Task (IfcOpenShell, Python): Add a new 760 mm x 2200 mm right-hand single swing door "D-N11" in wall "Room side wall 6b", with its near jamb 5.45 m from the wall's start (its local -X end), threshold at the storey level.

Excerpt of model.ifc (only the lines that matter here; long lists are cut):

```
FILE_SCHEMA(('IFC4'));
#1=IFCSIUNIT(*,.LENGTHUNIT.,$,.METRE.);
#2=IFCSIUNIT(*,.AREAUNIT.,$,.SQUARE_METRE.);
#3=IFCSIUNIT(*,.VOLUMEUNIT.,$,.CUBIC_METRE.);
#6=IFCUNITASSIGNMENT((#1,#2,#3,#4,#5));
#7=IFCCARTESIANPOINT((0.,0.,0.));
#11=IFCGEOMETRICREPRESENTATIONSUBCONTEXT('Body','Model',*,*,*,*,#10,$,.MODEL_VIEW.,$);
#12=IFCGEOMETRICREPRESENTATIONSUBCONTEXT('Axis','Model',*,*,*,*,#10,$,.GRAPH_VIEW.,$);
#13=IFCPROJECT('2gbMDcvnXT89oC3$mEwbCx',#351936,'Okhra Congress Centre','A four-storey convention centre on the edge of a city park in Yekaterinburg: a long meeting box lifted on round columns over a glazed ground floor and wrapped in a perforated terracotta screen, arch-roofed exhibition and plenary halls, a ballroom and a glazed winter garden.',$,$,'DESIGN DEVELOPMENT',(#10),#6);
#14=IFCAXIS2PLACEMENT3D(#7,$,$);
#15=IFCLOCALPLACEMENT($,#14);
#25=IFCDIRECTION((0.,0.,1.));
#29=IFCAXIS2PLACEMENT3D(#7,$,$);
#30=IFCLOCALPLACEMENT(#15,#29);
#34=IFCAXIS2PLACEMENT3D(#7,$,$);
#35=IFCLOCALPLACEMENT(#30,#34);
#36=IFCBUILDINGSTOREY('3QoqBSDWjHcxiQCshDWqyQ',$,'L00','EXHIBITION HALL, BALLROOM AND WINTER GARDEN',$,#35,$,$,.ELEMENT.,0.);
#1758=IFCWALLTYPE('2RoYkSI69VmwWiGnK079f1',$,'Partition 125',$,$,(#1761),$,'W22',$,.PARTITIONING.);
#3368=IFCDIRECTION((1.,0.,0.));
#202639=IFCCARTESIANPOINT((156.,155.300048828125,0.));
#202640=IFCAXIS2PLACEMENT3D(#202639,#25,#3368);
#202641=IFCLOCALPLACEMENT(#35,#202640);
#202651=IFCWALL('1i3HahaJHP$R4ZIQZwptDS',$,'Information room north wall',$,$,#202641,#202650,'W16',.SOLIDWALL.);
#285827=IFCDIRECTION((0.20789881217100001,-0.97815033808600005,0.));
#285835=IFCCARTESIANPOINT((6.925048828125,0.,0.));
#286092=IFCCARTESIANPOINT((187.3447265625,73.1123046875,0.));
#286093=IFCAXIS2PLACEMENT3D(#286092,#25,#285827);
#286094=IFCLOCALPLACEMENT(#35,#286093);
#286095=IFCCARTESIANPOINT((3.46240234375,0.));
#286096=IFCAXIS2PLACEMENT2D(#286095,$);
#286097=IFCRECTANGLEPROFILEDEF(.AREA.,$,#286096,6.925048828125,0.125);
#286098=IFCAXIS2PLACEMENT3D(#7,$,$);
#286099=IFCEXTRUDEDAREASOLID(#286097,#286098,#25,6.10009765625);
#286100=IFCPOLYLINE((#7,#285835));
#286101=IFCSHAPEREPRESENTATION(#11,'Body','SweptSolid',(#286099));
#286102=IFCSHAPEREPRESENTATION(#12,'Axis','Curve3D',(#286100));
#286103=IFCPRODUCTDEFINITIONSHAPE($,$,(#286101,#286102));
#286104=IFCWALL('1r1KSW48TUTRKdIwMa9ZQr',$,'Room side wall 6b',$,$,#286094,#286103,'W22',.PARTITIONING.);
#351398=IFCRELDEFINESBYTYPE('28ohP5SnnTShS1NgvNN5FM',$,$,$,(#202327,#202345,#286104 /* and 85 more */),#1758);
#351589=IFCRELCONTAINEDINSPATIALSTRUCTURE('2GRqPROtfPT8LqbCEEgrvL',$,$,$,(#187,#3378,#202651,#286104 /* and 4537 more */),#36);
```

```python
import numpy as np
import ifcopenshell
import ifcopenshell.api.feature
import ifcopenshell.api.geometry
import ifcopenshell.api.root
import ifcopenshell.api.spatial
import ifcopenshell.geom
import ifcopenshell.util.element
import ifcopenshell.util.placement
import ifcopenshell.util.representation
import ifcopenshell.util.shape
import ifcopenshell.util.unit

model = ifcopenshell.open("model.ifc")
unit_scale = ifcopenshell.util.unit.calculate_unit_scale(model)
settings = ifcopenshell.geom.settings()


def volume(element):
    """Net volume in cubic metres, openings subtracted."""
    shape = ifcopenshell.geom.create_shape(settings, element)
    return ifcopenshell.util.shape.get_volume(shape.geometry)


wall = model.by_guid("1r1KSW48TUTRKdIwMa9ZQr")
storey = ifcopenshell.util.element.get_container(wall, ifc_class="IfcBuildingStorey")
context = ifcopenshell.util.representation.get_context(model, "Model", "Body", "MODEL_VIEW")
before = volume(wall)

width, height, from_end, sill = 0.76, 2.2, 5.45, 0.0  # metres

# The wall runs along its own X axis, and the end named is its -X end.
wall_shape = ifcopenshell.geom.create_shape(settings, wall)
x, y, z = ifcopenshell.util.shape.get_vertices(wall_shape.geometry).T
start = x.min() + from_end
face, thickness = float(y.min()), float(y.max() - y.min())
wall_matrix = ifcopenshell.util.placement.get_local_placement(wall.ObjectPlacement)
level = ifcopenshell.util.placement.get_local_placement(storey.ObjectPlacement)[2, 3]


def in_wall(x, y):
    """Placement at x, y metres in the wall's axes, at sill height."""
    matrix = wall_matrix.copy()
    matrix[:, 3] = wall_matrix @ np.array([x / unit_scale, y / unit_scale, 0.0, 1.0])
    matrix[2, 3] = level + sill / unit_scale
    return matrix


# Opening: a box that overshoots both wall faces by 50 mm.
opening = ifcopenshell.api.root.create_entity(model, ifc_class="IfcOpeningElement", predefined_type="OPENING")
box = ifcopenshell.api.geometry.add_wall_representation(
    model, context=context, length=width, height=height, thickness=thickness + 0.1
)
ifcopenshell.api.geometry.assign_representation(model, product=opening, representation=box)
ifcopenshell.api.geometry.edit_object_placement(model, product=opening, matrix=in_wall(start, face - 0.05), is_si=False)
ifcopenshell.api.feature.add_feature(model, feature=opening, element=wall)

door = ifcopenshell.api.root.create_entity(model, ifc_class="IfcDoor", name="D-N11", predefined_type="DOOR")
door.OverallWidth, door.OverallHeight = width / unit_scale, height / unit_scale
door.OperationType = "SINGLE_SWING_RIGHT"
body = ifcopenshell.api.geometry.add_door_representation(
    model,
    context=context,
    overall_width=door.OverallWidth,
    overall_height=door.OverallHeight,
    operation_type="SINGLE_SWING_RIGHT",
    lining_properties={"LiningDepth": thickness / unit_scale, "ThresholdDepth": thickness / unit_scale},
)
ifcopenshell.api.geometry.assign_representation(model, product=door, representation=body)
ifcopenshell.api.spatial.assign_container(model, products=[door], relating_structure=storey)
ifcopenshell.api.feature.add_filling(model, opening=opening, element=door)

# The lining spans the wall, so the door starts at the wall face.
ifcopenshell.api.geometry.edit_object_placement(model, product=door, matrix=in_wall(start, face), is_si=False)

after = volume(wall)

print(f"wall volume {before:.3f} -> {after:.3f} m3")

model.write("model-out.ifc")
```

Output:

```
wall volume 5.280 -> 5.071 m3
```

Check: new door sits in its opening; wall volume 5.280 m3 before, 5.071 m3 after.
